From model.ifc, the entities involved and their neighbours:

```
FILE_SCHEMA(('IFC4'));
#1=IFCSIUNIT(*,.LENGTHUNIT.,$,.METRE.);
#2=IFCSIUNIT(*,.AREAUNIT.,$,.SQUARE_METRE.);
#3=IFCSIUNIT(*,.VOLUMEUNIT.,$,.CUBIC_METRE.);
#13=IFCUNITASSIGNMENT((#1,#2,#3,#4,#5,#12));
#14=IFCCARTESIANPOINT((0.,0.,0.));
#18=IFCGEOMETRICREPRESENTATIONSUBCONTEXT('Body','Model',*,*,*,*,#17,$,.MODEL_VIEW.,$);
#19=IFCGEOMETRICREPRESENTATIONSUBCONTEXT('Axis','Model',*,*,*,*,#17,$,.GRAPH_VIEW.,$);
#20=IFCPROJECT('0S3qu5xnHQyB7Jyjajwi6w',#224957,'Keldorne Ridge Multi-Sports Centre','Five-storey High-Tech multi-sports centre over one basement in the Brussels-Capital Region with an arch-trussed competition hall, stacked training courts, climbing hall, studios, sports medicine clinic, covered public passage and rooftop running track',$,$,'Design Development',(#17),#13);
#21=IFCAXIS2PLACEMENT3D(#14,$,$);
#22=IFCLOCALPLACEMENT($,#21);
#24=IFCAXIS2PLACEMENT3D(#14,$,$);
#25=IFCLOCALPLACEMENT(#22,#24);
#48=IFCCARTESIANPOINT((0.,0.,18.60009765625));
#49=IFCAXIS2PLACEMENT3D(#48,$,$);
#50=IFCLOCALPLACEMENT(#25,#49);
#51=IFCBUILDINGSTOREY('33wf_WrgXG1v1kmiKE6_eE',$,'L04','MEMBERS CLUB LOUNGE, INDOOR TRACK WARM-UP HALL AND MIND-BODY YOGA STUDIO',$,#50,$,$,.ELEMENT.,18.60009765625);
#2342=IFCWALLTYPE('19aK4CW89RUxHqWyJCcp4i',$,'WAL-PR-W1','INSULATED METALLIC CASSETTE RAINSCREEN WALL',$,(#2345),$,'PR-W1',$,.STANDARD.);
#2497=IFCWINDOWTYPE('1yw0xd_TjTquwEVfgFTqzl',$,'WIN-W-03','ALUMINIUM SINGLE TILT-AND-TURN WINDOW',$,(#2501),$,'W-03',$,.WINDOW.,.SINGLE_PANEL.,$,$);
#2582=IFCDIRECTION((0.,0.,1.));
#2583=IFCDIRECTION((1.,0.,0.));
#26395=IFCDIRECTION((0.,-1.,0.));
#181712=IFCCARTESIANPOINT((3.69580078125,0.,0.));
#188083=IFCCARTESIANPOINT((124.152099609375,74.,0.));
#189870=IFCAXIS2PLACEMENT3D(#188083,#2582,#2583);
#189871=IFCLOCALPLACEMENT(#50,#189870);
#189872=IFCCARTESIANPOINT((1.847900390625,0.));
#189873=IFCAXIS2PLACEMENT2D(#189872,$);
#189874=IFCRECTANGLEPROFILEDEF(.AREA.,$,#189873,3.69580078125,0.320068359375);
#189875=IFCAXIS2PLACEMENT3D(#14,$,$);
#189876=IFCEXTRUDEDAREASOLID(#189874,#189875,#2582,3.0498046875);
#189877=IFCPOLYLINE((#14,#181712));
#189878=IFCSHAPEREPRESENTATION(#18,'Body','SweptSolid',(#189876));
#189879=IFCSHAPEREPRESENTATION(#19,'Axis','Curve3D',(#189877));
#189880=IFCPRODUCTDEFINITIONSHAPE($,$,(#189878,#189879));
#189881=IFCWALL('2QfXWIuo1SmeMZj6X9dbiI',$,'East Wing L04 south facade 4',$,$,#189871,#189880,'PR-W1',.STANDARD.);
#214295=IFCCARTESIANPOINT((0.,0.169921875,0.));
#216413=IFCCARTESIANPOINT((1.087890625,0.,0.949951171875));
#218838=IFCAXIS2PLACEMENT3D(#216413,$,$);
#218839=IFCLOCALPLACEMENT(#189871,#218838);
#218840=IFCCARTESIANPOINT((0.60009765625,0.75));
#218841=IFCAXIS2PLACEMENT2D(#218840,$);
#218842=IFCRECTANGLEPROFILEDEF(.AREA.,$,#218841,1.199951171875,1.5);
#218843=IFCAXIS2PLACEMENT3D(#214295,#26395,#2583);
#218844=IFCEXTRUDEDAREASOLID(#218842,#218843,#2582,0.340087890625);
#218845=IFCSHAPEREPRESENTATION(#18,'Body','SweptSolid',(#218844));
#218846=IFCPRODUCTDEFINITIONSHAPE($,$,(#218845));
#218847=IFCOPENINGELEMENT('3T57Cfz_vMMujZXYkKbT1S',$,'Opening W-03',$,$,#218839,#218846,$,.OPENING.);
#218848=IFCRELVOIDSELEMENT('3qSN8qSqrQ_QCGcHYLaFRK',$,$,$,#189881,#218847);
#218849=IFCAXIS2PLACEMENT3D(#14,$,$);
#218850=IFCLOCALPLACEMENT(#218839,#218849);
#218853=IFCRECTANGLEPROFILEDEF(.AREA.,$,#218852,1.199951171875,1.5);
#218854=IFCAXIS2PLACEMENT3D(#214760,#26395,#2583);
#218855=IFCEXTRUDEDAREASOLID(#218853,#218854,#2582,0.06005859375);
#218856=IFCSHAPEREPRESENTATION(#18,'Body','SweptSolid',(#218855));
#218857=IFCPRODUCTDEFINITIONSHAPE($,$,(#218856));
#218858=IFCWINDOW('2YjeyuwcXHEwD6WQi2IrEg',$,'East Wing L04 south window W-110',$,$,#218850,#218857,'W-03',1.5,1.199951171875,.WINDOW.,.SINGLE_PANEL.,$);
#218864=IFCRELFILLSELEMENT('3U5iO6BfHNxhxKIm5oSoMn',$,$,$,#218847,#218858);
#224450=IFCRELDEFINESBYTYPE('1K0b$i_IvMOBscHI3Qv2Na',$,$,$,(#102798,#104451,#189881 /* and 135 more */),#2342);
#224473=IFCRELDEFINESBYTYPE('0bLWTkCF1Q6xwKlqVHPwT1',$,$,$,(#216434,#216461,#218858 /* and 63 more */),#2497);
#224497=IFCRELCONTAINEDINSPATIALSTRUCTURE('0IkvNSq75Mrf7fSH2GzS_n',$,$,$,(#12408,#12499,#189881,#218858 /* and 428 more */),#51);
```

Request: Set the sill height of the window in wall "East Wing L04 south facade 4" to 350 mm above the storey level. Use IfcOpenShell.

```python
import numpy as np
import ifcopenshell
import ifcopenshell.api.geometry
import ifcopenshell.geom
import ifcopenshell.util.element
import ifcopenshell.util.placement
import ifcopenshell.util.shape
import ifcopenshell.util.unit

model = ifcopenshell.open("model.ifc")
unit_scale = ifcopenshell.util.unit.calculate_unit_scale(model)

window = model.by_guid("2YjeyuwcXHEwD6WQi2IrEg")
opening = window.FillsVoids[0].RelatingOpeningElement
storey = ifcopenshell.util.element.get_container(window, ifc_class="IfcBuildingStorey")
level = ifcopenshell.util.placement.get_local_placement(storey.ObjectPlacement)[2, 3]

# The opening's origin need not be at the sill, so measure its lowest point.
shape = ifcopenshell.geom.create_shape(ifcopenshell.geom.settings(), opening)
bottom = ifcopenshell.util.shape.get_shape_bottom_elevation(shape, shape.geometry) / unit_scale
dz = level + 0.35 - bottom

shift = np.array([0.0, 0.0, dz])
# The window is placed relative to its opening, so it follows when the opening moves.
matrix = ifcopenshell.util.placement.get_local_placement(opening.ObjectPlacement)
matrix[:3, 3] += shift
ifcopenshell.api.geometry.edit_object_placement(
    model, product=opening, matrix=matrix, is_si=False, should_transform_children=True
)

print(f"moved by {dz * unit_scale:+.3f} m")

model.write("model_rev.ifc")
```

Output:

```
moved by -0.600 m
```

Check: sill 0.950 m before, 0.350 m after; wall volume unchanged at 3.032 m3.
